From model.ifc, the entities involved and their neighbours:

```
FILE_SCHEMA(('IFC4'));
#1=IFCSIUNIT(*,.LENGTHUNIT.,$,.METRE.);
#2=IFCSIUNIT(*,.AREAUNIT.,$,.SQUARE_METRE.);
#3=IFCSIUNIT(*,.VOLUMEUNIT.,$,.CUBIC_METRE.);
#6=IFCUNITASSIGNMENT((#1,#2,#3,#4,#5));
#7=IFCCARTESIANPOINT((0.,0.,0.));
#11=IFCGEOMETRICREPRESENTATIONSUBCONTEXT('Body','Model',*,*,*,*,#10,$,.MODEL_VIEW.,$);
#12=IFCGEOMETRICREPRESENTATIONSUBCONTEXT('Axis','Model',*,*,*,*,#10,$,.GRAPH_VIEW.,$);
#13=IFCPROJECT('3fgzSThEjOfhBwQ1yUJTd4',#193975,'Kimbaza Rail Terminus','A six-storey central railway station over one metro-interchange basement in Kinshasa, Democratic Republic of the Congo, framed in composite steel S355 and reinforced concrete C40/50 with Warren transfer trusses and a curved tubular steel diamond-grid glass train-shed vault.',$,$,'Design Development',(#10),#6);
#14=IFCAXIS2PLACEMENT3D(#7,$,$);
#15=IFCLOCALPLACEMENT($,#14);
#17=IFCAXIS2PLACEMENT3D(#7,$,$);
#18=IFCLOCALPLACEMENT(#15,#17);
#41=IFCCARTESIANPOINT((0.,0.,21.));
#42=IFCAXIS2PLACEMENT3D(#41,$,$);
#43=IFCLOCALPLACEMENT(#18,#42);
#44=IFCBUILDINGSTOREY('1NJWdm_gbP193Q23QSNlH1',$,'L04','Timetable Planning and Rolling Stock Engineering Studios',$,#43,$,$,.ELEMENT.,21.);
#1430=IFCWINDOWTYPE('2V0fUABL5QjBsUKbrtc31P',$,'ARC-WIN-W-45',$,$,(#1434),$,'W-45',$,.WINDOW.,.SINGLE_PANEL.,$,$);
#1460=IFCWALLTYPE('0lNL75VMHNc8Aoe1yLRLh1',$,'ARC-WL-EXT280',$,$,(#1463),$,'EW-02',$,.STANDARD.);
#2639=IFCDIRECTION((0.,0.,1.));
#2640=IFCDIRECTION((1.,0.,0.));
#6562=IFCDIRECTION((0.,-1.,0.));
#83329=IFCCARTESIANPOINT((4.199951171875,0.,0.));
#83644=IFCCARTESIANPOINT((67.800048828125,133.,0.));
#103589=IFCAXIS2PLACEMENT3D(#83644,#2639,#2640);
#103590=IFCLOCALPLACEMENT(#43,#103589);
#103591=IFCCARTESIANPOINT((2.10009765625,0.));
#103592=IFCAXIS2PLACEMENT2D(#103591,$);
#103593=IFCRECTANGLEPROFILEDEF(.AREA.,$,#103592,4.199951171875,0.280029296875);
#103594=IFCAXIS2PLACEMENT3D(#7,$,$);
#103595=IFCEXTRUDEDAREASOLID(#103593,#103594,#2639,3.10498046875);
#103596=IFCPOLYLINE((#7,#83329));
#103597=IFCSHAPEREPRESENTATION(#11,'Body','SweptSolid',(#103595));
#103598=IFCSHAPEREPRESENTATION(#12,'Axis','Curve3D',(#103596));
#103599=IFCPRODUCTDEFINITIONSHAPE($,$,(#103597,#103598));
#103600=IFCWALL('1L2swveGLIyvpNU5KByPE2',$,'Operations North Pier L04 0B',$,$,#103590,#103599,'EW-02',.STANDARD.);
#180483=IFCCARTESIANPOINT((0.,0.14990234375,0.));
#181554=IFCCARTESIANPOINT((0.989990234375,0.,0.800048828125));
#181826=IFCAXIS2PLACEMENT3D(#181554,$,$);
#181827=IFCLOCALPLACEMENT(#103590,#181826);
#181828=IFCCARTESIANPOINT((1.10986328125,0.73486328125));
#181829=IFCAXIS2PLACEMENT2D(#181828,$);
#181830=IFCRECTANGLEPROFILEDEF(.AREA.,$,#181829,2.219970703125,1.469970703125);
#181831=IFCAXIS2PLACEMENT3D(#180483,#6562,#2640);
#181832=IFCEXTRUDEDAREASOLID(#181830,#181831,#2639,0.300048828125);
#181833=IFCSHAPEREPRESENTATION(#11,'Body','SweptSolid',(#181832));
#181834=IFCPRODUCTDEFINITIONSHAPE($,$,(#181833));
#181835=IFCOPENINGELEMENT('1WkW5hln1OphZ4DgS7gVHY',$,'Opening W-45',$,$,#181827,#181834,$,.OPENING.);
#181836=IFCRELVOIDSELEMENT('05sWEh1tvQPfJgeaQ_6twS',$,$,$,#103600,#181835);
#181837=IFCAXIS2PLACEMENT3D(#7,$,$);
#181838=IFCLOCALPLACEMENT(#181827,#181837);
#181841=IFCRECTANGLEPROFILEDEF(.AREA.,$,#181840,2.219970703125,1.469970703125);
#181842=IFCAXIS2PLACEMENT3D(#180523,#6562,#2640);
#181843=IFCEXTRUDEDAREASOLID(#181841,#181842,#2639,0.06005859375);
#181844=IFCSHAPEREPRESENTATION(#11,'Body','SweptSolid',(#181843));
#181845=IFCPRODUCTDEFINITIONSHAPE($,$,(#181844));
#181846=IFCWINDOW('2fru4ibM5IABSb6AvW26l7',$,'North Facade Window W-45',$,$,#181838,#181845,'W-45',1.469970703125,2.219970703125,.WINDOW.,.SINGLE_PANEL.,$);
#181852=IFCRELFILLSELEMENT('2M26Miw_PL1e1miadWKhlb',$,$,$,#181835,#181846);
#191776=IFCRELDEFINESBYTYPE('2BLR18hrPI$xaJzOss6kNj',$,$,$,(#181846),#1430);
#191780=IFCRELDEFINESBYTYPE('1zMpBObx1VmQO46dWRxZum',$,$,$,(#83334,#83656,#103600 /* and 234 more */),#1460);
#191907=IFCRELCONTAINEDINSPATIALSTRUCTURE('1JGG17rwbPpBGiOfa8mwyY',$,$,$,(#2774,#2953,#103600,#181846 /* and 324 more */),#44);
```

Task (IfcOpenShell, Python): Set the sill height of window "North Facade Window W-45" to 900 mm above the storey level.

```python
import numpy as np
import ifcopenshell
import ifcopenshell.api.geometry
import ifcopenshell.geom
import ifcopenshell.util.element
import ifcopenshell.util.placement
import ifcopenshell.util.shape
import ifcopenshell.util.unit

model = ifcopenshell.open("model.ifc")
unit_scale = ifcopenshell.util.unit.calculate_unit_scale(model)

window = model.by_guid("2fru4ibM5IABSb6AvW26l7")
opening = window.FillsVoids[0].RelatingOpeningElement
storey = ifcopenshell.util.element.get_container(window, ifc_class="IfcBuildingStorey")
level = ifcopenshell.util.placement.get_local_placement(storey.ObjectPlacement)[2, 3]

# The opening's origin need not be at the sill, so measure its lowest point.
shape = ifcopenshell.geom.create_shape(ifcopenshell.geom.settings(), opening)
bottom = ifcopenshell.util.shape.get_shape_bottom_elevation(shape, shape.geometry) / unit_scale
dz = level + 0.9 / unit_scale - bottom

shift = np.array([0.0, 0.0, dz])
# The window is placed relative to its opening, so it follows when the opening moves.
matrix = ifcopenshell.util.placement.get_local_placement(opening.ObjectPlacement)
matrix[:3, 3] += shift
ifcopenshell.api.geometry.edit_object_placement(
    model, product=opening, matrix=matrix, is_si=False, should_transform_children=True
)

print(f"moved by {dz * unit_scale:+.3f} m")

model.write("model_rev.ifc")
```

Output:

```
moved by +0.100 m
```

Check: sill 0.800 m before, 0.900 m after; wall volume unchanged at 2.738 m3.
